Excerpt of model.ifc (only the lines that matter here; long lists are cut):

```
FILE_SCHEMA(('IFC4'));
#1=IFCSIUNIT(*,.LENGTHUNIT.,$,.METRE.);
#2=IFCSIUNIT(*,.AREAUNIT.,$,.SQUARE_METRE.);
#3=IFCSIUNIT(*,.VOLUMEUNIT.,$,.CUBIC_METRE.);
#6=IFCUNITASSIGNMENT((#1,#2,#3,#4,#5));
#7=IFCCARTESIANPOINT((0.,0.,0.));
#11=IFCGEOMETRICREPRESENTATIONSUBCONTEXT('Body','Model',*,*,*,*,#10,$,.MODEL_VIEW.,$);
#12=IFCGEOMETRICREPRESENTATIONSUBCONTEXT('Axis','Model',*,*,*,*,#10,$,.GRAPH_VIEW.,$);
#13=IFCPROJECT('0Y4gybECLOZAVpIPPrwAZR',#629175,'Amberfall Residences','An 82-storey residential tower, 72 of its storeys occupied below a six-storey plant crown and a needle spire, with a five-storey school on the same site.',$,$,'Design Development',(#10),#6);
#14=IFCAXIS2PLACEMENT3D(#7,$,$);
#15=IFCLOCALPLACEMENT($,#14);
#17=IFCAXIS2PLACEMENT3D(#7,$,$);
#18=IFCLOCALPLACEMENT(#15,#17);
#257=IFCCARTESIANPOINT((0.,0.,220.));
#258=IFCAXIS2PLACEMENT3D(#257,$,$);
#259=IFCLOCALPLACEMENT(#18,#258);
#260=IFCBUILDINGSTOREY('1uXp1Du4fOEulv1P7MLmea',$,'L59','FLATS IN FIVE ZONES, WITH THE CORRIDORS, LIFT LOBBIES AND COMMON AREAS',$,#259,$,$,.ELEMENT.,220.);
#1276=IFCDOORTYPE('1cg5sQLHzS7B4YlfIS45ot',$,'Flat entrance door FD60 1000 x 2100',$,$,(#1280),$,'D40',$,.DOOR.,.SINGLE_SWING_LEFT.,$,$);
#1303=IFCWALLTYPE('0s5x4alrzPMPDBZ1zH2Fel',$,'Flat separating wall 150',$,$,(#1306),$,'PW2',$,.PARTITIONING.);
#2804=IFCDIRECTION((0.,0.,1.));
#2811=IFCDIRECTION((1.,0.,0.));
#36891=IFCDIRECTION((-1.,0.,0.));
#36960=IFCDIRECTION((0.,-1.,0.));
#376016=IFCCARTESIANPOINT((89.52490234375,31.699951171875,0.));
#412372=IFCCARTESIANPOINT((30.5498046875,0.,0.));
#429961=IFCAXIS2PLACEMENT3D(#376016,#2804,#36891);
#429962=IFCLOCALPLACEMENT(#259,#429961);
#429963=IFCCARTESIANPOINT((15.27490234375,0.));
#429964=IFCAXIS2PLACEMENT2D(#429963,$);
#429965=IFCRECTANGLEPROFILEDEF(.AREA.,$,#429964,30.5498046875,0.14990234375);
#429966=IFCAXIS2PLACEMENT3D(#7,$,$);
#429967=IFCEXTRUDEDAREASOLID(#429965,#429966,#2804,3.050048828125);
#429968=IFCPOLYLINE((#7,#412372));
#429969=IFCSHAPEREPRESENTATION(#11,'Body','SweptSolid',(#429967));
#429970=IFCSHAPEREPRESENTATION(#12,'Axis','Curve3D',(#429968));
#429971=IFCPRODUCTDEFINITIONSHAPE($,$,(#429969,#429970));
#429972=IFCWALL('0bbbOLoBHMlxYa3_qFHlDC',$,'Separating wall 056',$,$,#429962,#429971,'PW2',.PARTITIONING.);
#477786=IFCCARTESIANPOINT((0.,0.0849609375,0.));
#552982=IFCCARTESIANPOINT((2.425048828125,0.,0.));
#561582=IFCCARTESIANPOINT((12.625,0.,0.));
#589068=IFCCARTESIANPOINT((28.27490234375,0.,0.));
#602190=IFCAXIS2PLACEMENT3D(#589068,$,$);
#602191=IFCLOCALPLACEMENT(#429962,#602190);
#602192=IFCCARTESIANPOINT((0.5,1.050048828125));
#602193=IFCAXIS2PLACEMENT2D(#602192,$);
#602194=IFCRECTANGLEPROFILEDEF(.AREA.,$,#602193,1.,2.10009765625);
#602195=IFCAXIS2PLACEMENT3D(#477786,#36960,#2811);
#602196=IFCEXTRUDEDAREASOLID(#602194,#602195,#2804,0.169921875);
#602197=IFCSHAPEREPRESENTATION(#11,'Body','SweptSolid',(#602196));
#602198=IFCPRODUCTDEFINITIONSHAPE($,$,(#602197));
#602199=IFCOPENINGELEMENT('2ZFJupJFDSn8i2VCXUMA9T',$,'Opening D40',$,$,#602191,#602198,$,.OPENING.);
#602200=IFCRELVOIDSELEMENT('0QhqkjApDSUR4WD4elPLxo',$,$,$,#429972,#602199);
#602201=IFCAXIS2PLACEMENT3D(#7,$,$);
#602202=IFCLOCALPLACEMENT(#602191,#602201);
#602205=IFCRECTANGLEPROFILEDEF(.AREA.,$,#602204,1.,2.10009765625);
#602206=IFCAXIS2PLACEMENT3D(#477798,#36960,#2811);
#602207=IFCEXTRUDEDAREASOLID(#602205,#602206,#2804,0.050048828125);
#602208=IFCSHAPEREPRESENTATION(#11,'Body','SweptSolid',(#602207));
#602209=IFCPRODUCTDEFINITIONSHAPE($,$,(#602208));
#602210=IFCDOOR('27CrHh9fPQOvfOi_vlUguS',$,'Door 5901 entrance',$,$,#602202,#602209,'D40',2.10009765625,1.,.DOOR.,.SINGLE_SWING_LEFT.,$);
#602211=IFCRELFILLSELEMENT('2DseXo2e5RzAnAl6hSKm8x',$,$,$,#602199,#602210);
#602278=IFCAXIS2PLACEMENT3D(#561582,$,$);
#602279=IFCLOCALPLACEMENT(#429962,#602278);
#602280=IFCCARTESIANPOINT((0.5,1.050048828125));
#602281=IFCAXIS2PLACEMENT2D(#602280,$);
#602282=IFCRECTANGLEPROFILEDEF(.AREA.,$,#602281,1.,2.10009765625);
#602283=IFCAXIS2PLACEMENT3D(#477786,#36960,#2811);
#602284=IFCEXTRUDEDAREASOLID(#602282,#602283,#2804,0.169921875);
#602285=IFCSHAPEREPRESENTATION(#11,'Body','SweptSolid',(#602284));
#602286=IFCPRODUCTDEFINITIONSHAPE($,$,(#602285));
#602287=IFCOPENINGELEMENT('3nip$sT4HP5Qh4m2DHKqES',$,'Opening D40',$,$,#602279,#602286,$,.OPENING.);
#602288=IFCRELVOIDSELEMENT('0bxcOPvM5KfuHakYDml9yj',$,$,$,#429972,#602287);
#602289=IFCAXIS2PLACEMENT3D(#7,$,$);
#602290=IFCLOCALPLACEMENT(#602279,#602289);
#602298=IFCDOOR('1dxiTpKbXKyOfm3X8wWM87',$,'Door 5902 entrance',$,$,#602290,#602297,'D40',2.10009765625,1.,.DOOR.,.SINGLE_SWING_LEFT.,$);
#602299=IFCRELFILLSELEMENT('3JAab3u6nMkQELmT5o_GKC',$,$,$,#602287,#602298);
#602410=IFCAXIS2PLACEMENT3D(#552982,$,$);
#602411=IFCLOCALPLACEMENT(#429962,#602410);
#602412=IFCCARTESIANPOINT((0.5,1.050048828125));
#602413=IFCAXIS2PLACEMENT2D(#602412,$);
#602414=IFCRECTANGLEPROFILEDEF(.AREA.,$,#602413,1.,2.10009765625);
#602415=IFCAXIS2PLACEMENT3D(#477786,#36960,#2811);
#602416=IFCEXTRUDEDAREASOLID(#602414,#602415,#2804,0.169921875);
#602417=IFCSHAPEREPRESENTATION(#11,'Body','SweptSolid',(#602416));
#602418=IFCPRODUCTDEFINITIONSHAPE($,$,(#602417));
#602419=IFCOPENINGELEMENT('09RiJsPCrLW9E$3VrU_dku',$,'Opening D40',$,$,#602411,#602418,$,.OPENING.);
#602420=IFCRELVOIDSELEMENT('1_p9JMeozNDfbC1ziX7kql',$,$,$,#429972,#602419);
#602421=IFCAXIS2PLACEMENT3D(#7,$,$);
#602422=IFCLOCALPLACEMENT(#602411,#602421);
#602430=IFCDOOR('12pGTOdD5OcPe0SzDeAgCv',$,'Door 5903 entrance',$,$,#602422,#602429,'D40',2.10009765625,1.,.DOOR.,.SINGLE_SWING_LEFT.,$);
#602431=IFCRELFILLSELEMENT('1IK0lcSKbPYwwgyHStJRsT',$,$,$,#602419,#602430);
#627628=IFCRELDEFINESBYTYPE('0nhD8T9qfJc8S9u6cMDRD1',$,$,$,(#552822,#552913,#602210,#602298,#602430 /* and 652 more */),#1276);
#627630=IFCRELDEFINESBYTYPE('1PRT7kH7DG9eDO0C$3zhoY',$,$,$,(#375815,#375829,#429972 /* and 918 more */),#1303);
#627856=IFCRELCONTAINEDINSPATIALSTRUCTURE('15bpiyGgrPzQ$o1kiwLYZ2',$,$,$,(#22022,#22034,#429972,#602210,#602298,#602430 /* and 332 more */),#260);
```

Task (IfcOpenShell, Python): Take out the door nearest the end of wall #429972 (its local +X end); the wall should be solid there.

```python
import ifcopenshell
import ifcopenshell.api.feature
import ifcopenshell.api.root
import ifcopenshell.geom
import ifcopenshell.util.shape

model = ifcopenshell.open("model.ifc")
settings = ifcopenshell.geom.settings()


def volume(element):
    """Net volume in cubic metres, openings subtracted."""
    shape = ifcopenshell.geom.create_shape(settings, element)
    return ifcopenshell.util.shape.get_volume(shape.geometry)


door = model.by_id(602210)
opening = door.FillsVoids[0].RelatingOpeningElement
wall = opening.VoidsElements[0].RelatingBuildingElement
before = volume(wall)

ifcopenshell.api.root.remove_product(model, product=door)
ifcopenshell.api.feature.remove_feature(model, feature=opening)

after = volume(wall)

print(f"wall volume {before:.3f} -> {after:.3f} m3")

model.write("model_rev.ifc")
```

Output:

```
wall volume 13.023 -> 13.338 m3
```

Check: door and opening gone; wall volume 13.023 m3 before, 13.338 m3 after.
